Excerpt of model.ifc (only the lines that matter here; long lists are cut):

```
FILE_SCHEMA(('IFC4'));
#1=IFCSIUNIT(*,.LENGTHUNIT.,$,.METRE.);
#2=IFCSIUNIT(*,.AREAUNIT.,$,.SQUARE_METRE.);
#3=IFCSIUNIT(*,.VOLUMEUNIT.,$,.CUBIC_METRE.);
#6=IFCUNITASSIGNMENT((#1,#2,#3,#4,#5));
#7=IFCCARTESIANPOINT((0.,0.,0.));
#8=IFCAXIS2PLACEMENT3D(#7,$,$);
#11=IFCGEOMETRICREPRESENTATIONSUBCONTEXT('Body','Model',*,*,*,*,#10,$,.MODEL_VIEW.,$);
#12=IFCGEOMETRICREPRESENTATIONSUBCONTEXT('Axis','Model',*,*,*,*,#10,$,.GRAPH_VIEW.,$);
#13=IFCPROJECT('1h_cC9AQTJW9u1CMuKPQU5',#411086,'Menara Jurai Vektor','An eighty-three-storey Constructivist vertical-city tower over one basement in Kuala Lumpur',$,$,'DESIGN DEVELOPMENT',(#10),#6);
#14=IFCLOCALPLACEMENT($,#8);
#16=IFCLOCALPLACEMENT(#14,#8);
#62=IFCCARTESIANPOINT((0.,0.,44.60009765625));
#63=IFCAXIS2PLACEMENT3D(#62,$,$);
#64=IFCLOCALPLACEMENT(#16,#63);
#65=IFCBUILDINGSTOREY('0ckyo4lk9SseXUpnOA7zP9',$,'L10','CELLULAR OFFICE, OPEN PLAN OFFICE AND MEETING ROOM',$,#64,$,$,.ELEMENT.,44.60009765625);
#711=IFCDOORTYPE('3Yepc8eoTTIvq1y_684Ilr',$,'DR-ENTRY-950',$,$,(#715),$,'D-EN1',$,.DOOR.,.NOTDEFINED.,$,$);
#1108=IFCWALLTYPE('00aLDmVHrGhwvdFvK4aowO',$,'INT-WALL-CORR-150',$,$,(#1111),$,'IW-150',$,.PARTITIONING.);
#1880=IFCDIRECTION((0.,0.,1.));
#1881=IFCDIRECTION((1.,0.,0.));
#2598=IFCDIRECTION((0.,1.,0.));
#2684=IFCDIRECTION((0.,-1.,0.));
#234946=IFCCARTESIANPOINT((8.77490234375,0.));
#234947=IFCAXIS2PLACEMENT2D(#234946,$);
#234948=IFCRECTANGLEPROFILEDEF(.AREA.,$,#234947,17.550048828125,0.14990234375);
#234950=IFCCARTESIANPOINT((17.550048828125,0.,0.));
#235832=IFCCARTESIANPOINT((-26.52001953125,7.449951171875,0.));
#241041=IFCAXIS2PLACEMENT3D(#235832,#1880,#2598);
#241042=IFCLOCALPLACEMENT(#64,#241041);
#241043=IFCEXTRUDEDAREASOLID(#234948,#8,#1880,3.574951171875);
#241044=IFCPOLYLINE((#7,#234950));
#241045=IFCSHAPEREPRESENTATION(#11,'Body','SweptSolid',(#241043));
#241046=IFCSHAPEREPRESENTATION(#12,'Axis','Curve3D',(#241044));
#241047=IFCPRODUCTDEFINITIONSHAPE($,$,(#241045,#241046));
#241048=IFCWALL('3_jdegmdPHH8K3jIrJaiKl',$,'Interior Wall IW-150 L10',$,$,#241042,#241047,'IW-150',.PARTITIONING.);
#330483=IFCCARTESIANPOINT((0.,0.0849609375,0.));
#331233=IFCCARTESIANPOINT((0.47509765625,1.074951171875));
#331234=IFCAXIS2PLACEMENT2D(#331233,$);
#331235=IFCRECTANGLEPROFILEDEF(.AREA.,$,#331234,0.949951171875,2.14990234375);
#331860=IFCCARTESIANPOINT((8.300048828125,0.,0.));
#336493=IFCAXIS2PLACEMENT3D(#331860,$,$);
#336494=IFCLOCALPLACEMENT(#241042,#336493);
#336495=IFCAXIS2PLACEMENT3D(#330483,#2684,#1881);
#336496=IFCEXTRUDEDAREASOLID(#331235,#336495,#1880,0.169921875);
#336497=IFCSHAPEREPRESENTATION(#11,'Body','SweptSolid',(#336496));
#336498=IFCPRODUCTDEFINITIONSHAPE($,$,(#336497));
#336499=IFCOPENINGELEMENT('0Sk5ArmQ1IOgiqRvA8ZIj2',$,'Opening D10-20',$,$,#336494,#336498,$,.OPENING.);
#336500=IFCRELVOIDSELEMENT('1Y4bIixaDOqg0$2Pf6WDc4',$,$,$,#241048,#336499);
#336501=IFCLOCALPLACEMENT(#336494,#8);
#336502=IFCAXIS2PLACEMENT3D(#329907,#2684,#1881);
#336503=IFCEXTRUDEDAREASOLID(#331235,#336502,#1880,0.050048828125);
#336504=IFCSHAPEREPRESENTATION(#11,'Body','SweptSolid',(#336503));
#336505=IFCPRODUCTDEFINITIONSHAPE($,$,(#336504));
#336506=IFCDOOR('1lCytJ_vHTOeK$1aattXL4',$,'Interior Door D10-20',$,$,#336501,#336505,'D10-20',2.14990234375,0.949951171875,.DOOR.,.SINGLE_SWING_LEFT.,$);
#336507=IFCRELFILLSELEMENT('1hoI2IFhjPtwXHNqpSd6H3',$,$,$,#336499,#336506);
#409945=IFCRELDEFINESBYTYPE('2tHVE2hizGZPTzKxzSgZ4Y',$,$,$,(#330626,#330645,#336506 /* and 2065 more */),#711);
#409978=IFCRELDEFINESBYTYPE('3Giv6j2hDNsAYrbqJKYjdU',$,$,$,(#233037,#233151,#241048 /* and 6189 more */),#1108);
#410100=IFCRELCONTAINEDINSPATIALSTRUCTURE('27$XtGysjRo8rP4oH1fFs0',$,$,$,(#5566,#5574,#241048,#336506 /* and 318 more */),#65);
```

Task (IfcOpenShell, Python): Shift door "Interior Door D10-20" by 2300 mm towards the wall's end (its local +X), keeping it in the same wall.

```python
import ifcopenshell
import ifcopenshell.api.geometry
import ifcopenshell.util.placement
import ifcopenshell.util.unit

model = ifcopenshell.open("model.ifc")
unit_scale = ifcopenshell.util.unit.calculate_unit_scale(model)

door = model.by_guid("1lCytJ_vHTOeK$1aattXL4")
opening = door.FillsVoids[0].RelatingOpeningElement
wall = opening.VoidsElements[0].RelatingBuildingElement

wall_matrix = ifcopenshell.util.placement.get_local_placement(wall.ObjectPlacement)
shift = wall_matrix[:3, 0] * 2.3 / unit_scale
before = ifcopenshell.util.placement.get_local_placement(door.ObjectPlacement)[:3, 3].copy()

# The door is placed relative to its opening, so it follows when the opening moves.
matrix = ifcopenshell.util.placement.get_local_placement(opening.ObjectPlacement)
matrix[:3, 3] += shift
ifcopenshell.api.geometry.edit_object_placement(
    model, product=opening, matrix=matrix, is_si=False, should_transform_children=True
)

after = ifcopenshell.util.placement.get_local_placement(door.ObjectPlacement)[:3, 3]
print("door moved by", (after - before).round(3) + 0.0)

model.write("model-out.ifc")
```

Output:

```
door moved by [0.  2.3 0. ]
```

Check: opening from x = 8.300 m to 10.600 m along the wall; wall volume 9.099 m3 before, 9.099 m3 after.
